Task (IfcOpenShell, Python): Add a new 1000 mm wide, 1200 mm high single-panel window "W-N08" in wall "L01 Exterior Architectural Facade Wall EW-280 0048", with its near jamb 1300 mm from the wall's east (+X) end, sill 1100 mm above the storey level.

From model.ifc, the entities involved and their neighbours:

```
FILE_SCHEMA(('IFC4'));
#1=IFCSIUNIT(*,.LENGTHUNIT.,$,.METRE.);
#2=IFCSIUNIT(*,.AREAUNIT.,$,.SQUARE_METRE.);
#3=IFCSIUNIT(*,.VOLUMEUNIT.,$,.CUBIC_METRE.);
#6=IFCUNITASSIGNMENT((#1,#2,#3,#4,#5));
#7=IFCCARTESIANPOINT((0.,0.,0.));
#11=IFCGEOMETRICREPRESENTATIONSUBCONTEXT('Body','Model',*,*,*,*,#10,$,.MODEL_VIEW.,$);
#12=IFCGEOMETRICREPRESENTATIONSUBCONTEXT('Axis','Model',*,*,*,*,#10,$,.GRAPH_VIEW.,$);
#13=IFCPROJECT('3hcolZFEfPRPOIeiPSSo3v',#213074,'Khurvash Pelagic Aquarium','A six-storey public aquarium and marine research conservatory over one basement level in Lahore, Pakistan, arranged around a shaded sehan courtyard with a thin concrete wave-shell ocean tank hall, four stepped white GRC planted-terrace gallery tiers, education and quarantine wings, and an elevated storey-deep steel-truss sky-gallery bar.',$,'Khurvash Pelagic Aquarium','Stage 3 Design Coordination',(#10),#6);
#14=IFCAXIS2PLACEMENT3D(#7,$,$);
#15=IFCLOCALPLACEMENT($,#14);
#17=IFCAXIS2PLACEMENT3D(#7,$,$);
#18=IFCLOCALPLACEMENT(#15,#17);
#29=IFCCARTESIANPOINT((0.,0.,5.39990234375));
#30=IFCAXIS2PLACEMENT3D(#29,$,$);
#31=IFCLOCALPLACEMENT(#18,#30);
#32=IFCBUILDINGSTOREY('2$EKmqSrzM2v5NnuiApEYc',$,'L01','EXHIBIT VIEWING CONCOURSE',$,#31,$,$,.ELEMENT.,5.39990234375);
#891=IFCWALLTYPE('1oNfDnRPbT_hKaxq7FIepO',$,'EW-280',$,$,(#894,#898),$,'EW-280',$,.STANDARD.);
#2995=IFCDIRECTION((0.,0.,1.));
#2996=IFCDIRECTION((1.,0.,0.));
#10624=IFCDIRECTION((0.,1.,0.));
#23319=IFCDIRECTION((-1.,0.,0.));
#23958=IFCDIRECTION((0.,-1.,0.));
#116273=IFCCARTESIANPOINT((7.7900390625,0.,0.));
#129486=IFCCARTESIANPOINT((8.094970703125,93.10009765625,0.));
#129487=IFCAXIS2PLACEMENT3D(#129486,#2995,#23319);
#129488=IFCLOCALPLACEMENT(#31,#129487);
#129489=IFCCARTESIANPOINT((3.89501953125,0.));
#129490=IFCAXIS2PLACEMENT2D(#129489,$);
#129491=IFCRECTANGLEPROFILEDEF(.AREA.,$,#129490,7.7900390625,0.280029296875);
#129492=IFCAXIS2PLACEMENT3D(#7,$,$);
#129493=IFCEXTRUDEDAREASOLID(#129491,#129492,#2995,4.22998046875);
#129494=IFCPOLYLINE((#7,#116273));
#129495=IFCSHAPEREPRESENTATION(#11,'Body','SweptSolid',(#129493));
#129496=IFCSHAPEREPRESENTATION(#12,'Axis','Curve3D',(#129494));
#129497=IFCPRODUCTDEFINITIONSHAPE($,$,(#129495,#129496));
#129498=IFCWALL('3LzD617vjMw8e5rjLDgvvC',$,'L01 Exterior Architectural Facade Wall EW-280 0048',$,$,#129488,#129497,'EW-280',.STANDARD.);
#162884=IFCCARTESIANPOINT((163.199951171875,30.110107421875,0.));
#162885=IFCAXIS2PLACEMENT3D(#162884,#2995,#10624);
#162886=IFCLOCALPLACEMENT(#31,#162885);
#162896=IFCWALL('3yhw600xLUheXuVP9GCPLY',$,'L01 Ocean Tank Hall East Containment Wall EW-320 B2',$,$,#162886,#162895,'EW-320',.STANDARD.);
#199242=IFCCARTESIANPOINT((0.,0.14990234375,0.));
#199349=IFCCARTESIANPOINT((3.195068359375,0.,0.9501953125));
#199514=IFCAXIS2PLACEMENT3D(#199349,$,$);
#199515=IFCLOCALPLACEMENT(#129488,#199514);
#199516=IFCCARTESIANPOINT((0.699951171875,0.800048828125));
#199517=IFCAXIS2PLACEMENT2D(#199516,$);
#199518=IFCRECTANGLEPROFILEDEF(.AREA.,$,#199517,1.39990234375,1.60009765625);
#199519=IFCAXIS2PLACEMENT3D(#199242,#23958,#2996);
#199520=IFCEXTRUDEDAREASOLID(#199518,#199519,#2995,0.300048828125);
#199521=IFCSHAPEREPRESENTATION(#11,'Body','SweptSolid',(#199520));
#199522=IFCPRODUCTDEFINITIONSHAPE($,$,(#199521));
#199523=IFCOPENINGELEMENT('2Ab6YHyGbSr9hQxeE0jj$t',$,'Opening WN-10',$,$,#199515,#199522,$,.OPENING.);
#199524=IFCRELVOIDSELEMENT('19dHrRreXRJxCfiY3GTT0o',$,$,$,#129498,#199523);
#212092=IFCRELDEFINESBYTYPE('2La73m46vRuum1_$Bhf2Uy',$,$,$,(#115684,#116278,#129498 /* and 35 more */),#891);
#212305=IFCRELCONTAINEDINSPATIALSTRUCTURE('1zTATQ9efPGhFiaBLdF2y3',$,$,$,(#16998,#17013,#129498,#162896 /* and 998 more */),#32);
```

```python
import numpy as np
import ifcopenshell
import ifcopenshell.api.feature
import ifcopenshell.api.geometry
import ifcopenshell.api.root
import ifcopenshell.api.spatial
import ifcopenshell.geom
import ifcopenshell.util.element
import ifcopenshell.util.placement
import ifcopenshell.util.representation
import ifcopenshell.util.shape
import ifcopenshell.util.unit

model = ifcopenshell.open("model.ifc")
unit_scale = ifcopenshell.util.unit.calculate_unit_scale(model)
settings = ifcopenshell.geom.settings()


def volume(element):
    """Net volume in cubic metres, openings subtracted."""
    shape = ifcopenshell.geom.create_shape(settings, element)
    return ifcopenshell.util.shape.get_volume(shape.geometry)


wall = model.by_guid("3LzD617vjMw8e5rjLDgvvC")
storey = ifcopenshell.util.element.get_container(wall, ifc_class="IfcBuildingStorey")
context = ifcopenshell.util.representation.get_context(model, "Model", "Body", "MODEL_VIEW")
before = volume(wall)

width, height, from_end, sill = 1, 1.2, 1.3, 1.1  # metres

# The wall runs along its own X axis, and the end named is its -X end.
wall_shape = ifcopenshell.geom.create_shape(settings, wall)
x, y, z = ifcopenshell.util.shape.get_vertices(wall_shape.geometry).T
start = x.min() + from_end
face, thickness = float(y.min()), float(y.max() - y.min())
wall_matrix = ifcopenshell.util.placement.get_local_placement(wall.ObjectPlacement)
level = ifcopenshell.util.placement.get_local_placement(storey.ObjectPlacement)[2, 3]


def in_wall(x, y):
    """Placement at x, y metres in the wall's axes, at sill height."""
    matrix = wall_matrix.copy()
    matrix[:, 3] = wall_matrix @ np.array([x / unit_scale, y / unit_scale, 0.0, 1.0])
    matrix[2, 3] = level + sill / unit_scale
    return matrix


# Opening: a box that overshoots both wall faces by 50 mm.
opening = ifcopenshell.api.root.create_entity(model, ifc_class="IfcOpeningElement", predefined_type="OPENING")
box = ifcopenshell.api.geometry.add_wall_representation(
    model, context=context, length=width, height=height, thickness=thickness + 0.1
)
ifcopenshell.api.geometry.assign_representation(model, product=opening, representation=box)
ifcopenshell.api.geometry.edit_object_placement(model, product=opening, matrix=in_wall(start, face - 0.05), is_si=False)
ifcopenshell.api.feature.add_feature(model, feature=opening, element=wall)

window = ifcopenshell.api.root.create_entity(model, ifc_class="IfcWindow", name="W-N08", predefined_type="WINDOW")
window.OverallWidth, window.OverallHeight = width / unit_scale, height / unit_scale
window.PartitioningType = "SINGLE_PANEL"
body = ifcopenshell.api.geometry.add_window_representation(
    model,
    context=context,
    overall_width=window.OverallWidth,
    overall_height=window.OverallHeight,
    partition_type="SINGLE_PANEL",
)
ifcopenshell.api.geometry.assign_representation(model, product=window, representation=body)
ifcopenshell.api.spatial.assign_container(model, products=[window], relating_structure=storey)
ifcopenshell.api.feature.add_filling(model, opening=opening, element=window)

# Centre the window in the wall's thickness.
ifcopenshell.api.geometry.edit_object_placement(model, product=window, matrix=in_wall(start, face), is_si=False)
window_shape = ifcopenshell.geom.create_shape(settings, window)
depth = ifcopenshell.util.shape.get_vertices(window_shape.geometry)[:, 1]
offset = face + thickness / 2 - (depth.min() + depth.max()) / 2
ifcopenshell.api.geometry.edit_object_placement(model, product=window, matrix=in_wall(start, offset), is_si=False)

after = volume(wall)

print(f"wall volume {before:.3f} -> {after:.3f} m3")

model.write("model-out.ifc")
```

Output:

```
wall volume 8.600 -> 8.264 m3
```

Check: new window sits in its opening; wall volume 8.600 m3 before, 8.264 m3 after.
